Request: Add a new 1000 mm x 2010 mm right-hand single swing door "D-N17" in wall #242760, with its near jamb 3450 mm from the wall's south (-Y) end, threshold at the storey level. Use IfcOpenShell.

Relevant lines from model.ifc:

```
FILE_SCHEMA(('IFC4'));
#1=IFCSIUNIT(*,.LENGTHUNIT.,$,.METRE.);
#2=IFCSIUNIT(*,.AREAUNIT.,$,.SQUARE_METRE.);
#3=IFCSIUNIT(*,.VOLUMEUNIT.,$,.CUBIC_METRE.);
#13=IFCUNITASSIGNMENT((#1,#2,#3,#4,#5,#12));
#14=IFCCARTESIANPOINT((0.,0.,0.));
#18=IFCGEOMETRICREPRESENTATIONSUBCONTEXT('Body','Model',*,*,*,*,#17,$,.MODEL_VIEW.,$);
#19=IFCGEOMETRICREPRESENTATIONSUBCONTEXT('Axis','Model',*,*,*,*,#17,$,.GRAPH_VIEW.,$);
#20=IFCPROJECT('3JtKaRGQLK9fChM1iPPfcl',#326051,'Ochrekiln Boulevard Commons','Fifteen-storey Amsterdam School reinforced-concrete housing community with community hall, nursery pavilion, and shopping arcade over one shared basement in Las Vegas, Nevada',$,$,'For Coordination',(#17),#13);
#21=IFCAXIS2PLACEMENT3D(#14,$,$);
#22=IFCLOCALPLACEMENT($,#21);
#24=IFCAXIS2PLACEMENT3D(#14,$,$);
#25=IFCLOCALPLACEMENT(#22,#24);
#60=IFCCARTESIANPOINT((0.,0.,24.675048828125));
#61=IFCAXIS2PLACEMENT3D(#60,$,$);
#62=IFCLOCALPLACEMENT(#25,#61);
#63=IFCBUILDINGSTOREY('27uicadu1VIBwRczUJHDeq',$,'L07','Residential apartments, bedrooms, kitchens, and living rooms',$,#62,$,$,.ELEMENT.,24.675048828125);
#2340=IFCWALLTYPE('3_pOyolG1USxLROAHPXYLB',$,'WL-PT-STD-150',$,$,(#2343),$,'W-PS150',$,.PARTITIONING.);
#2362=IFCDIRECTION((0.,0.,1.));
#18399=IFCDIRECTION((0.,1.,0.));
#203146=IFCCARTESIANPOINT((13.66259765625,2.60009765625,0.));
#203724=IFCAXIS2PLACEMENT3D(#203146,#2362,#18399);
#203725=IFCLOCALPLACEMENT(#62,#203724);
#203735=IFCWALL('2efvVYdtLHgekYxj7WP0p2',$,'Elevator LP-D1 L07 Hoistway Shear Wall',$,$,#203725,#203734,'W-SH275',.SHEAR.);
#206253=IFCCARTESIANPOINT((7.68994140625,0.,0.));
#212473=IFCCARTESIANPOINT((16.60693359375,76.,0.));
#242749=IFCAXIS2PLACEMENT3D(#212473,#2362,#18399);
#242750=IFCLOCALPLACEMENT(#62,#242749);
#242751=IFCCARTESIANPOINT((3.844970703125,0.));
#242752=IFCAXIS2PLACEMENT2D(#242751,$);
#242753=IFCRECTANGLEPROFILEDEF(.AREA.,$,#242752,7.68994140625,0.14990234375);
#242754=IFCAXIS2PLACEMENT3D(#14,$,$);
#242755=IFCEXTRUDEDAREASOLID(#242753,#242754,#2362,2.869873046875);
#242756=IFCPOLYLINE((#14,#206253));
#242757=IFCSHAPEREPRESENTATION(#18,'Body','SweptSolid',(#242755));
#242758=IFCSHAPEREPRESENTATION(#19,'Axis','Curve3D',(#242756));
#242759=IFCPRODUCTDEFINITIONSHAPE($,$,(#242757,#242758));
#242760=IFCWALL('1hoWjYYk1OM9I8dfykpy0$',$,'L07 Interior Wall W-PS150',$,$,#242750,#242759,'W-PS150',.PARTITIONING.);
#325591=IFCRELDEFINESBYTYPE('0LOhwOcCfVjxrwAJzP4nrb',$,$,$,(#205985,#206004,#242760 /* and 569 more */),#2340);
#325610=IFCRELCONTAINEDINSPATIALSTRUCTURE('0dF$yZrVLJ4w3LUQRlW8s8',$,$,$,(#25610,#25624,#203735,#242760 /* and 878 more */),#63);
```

```python
import numpy as np
import ifcopenshell
import ifcopenshell.api.feature
import ifcopenshell.api.geometry
import ifcopenshell.api.root
import ifcopenshell.api.spatial
import ifcopenshell.geom
import ifcopenshell.util.element
import ifcopenshell.util.placement
import ifcopenshell.util.representation
import ifcopenshell.util.shape
import ifcopenshell.util.unit

model = ifcopenshell.open("model.ifc")
unit_scale = ifcopenshell.util.unit.calculate_unit_scale(model)
settings = ifcopenshell.geom.settings()


def volume(element):
    """Net volume in cubic metres, openings subtracted."""
    shape = ifcopenshell.geom.create_shape(settings, element)
    return ifcopenshell.util.shape.get_volume(shape.geometry)


wall = model.by_guid("1hoWjYYk1OM9I8dfykpy0$")
storey = ifcopenshell.util.element.get_container(wall, ifc_class="IfcBuildingStorey")
context = ifcopenshell.util.representation.get_context(model, "Model", "Body", "MODEL_VIEW")
before = volume(wall)

width, height, from_end, sill = 1, 2.01, 3.45, 0.0  # metres

# The wall runs along its own X axis, and the end named is its -X end.
wall_shape = ifcopenshell.geom.create_shape(settings, wall)
x, y, z = ifcopenshell.util.shape.get_vertices(wall_shape.geometry).T
start = x.min() + from_end
face, thickness = float(y.min()), float(y.max() - y.min())
wall_matrix = ifcopenshell.util.placement.get_local_placement(wall.ObjectPlacement)
level = ifcopenshell.util.placement.get_local_placement(storey.ObjectPlacement)[2, 3]


def in_wall(x, y):
    """Placement at x, y metres in the wall's axes, at sill height."""
    matrix = wall_matrix.copy()
    matrix[:, 3] = wall_matrix @ np.array([x / unit_scale, y / unit_scale, 0.0, 1.0])
    matrix[2, 3] = level + sill / unit_scale
    return matrix


# Opening: a box that overshoots both wall faces by 50 mm.
opening = ifcopenshell.api.root.create_entity(model, ifc_class="IfcOpeningElement", predefined_type="OPENING")
box = ifcopenshell.api.geometry.add_wall_representation(
    model, context=context, length=width, height=height, thickness=thickness + 0.1
)
ifcopenshell.api.geometry.assign_representation(model, product=opening, representation=box)
ifcopenshell.api.geometry.edit_object_placement(model, product=opening, matrix=in_wall(start, face - 0.05), is_si=False)
ifcopenshell.api.feature.add_feature(model, feature=opening, element=wall)

door = ifcopenshell.api.root.create_entity(model, ifc_class="IfcDoor", name="D-N17", predefined_type="DOOR")
door.OverallWidth, door.OverallHeight = width / unit_scale, height / unit_scale
door.OperationType = "SINGLE_SWING_RIGHT"
body = ifcopenshell.api.geometry.add_door_representation(
    model,
    context=context,
    overall_width=door.OverallWidth,
    overall_height=door.OverallHeight,
    operation_type="SINGLE_SWING_RIGHT",
    lining_properties={"LiningDepth": thickness / unit_scale, "ThresholdDepth": thickness / unit_scale},
)
ifcopenshell.api.geometry.assign_representation(model, product=door, representation=body)
ifcopenshell.api.spatial.assign_container(model, products=[door], relating_structure=storey)
ifcopenshell.api.feature.add_filling(model, opening=opening, element=door)

# The lining spans the wall, so the door starts at the wall face.
ifcopenshell.api.geometry.edit_object_placement(model, product=door, matrix=in_wall(start, face), is_si=False)

after = volume(wall)

print(f"wall volume {before:.3f} -> {after:.3f} m3")

model.write("model_edited.ifc")
```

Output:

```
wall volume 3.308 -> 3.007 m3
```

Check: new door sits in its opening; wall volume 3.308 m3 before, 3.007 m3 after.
